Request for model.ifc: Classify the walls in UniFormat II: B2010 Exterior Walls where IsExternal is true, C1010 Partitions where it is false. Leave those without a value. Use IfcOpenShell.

First a look at what the model holds.

```python
import ifcopenshell
import ifcopenshell.util.element

model = ifcopenshell.open("model.ifc")
print(model.schema)
print("classifications:", [c.Name for c in model.by_type("IfcClassification")])
values = [ifcopenshell.util.element.get_pset(e, "Pset_WallCommon", "IsExternal") for e in model.by_type("IfcWall")]
for value in (True, False, None):
    print("IsExternal", value, values.count(value))
```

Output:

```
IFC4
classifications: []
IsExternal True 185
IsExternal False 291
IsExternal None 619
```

```python
import ifcopenshell
import ifcopenshell.api.classification
import ifcopenshell.util.element

model = ifcopenshell.open("model.ifc")

system = ifcopenshell.api.classification.add_classification(model, classification="UniFormat II")

walls = model.by_type("IfcWall")
external = {e: ifcopenshell.util.element.get_pset(e, "Pset_WallCommon", "IsExternal") for e in walls}
for flag, code, name in ((True, "B2010", "Exterior Walls"), (False, "C1010", "Partitions")):
    products = [e for e in walls if external[e] is flag]
    ifcopenshell.api.classification.add_reference(
        model, products=products, classification=system, identification=code, name=name
    )
    print(code, len(products))

model.write("model_updated.ifc")
```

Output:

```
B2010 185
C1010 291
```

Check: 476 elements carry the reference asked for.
